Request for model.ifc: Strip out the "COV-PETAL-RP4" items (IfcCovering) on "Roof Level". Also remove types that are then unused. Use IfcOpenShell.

First a look at what the model holds.

```python
import ifcopenshell
import ifcopenshell.util.element

model = ifcopenshell.open("model.ifc")
print(model.schema)
storey = next(s for s in model.by_type("IfcBuildingStorey") if s.Name == "Roof Level")
coverings = [e for e in ifcopenshell.util.element.get_decomposition(storey) if e.is_a("IfcCovering")]
seen = {}
for e in coverings:
    element_type = ifcopenshell.util.element.get_type(e)
    name = element_type.Name if element_type not in (None, e) else None
    seen[name] = seen.get(name, 0) + 1
for name, count in sorted(seen.items(), key=str):
    print(count, "x", name)
```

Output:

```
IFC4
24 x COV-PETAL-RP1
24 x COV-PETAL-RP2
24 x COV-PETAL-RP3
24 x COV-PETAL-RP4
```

```python
import ifcopenshell
import ifcopenshell.api.root
import ifcopenshell.util.element

model = ifcopenshell.open("model.ifc")

storey = next(s for s in model.by_type("IfcBuildingStorey") if s.Name == "Roof Level")
coverings = [e for e in ifcopenshell.util.element.get_decomposition(storey) if e.is_a("IfcCovering")]
targets = [e for e in coverings if (t := ifcopenshell.util.element.get_type(e)) not in (None, e) and t.Name == "COV-PETAL-RP4"]
types = {ifcopenshell.util.element.get_type(e) for e in targets} - {None, *targets}

for e in targets:
    ifcopenshell.api.root.remove_product(model, product=e)
print(len(targets), "removed")

unused = [t for t in types if not ifcopenshell.util.element.get_types(t)]
for t in unused:
    ifcopenshell.api.root.remove_product(model, product=t)
print(len(unused), "unused types removed")

model.write("model_updated.ifc")
```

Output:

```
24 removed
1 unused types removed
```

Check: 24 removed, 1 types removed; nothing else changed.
